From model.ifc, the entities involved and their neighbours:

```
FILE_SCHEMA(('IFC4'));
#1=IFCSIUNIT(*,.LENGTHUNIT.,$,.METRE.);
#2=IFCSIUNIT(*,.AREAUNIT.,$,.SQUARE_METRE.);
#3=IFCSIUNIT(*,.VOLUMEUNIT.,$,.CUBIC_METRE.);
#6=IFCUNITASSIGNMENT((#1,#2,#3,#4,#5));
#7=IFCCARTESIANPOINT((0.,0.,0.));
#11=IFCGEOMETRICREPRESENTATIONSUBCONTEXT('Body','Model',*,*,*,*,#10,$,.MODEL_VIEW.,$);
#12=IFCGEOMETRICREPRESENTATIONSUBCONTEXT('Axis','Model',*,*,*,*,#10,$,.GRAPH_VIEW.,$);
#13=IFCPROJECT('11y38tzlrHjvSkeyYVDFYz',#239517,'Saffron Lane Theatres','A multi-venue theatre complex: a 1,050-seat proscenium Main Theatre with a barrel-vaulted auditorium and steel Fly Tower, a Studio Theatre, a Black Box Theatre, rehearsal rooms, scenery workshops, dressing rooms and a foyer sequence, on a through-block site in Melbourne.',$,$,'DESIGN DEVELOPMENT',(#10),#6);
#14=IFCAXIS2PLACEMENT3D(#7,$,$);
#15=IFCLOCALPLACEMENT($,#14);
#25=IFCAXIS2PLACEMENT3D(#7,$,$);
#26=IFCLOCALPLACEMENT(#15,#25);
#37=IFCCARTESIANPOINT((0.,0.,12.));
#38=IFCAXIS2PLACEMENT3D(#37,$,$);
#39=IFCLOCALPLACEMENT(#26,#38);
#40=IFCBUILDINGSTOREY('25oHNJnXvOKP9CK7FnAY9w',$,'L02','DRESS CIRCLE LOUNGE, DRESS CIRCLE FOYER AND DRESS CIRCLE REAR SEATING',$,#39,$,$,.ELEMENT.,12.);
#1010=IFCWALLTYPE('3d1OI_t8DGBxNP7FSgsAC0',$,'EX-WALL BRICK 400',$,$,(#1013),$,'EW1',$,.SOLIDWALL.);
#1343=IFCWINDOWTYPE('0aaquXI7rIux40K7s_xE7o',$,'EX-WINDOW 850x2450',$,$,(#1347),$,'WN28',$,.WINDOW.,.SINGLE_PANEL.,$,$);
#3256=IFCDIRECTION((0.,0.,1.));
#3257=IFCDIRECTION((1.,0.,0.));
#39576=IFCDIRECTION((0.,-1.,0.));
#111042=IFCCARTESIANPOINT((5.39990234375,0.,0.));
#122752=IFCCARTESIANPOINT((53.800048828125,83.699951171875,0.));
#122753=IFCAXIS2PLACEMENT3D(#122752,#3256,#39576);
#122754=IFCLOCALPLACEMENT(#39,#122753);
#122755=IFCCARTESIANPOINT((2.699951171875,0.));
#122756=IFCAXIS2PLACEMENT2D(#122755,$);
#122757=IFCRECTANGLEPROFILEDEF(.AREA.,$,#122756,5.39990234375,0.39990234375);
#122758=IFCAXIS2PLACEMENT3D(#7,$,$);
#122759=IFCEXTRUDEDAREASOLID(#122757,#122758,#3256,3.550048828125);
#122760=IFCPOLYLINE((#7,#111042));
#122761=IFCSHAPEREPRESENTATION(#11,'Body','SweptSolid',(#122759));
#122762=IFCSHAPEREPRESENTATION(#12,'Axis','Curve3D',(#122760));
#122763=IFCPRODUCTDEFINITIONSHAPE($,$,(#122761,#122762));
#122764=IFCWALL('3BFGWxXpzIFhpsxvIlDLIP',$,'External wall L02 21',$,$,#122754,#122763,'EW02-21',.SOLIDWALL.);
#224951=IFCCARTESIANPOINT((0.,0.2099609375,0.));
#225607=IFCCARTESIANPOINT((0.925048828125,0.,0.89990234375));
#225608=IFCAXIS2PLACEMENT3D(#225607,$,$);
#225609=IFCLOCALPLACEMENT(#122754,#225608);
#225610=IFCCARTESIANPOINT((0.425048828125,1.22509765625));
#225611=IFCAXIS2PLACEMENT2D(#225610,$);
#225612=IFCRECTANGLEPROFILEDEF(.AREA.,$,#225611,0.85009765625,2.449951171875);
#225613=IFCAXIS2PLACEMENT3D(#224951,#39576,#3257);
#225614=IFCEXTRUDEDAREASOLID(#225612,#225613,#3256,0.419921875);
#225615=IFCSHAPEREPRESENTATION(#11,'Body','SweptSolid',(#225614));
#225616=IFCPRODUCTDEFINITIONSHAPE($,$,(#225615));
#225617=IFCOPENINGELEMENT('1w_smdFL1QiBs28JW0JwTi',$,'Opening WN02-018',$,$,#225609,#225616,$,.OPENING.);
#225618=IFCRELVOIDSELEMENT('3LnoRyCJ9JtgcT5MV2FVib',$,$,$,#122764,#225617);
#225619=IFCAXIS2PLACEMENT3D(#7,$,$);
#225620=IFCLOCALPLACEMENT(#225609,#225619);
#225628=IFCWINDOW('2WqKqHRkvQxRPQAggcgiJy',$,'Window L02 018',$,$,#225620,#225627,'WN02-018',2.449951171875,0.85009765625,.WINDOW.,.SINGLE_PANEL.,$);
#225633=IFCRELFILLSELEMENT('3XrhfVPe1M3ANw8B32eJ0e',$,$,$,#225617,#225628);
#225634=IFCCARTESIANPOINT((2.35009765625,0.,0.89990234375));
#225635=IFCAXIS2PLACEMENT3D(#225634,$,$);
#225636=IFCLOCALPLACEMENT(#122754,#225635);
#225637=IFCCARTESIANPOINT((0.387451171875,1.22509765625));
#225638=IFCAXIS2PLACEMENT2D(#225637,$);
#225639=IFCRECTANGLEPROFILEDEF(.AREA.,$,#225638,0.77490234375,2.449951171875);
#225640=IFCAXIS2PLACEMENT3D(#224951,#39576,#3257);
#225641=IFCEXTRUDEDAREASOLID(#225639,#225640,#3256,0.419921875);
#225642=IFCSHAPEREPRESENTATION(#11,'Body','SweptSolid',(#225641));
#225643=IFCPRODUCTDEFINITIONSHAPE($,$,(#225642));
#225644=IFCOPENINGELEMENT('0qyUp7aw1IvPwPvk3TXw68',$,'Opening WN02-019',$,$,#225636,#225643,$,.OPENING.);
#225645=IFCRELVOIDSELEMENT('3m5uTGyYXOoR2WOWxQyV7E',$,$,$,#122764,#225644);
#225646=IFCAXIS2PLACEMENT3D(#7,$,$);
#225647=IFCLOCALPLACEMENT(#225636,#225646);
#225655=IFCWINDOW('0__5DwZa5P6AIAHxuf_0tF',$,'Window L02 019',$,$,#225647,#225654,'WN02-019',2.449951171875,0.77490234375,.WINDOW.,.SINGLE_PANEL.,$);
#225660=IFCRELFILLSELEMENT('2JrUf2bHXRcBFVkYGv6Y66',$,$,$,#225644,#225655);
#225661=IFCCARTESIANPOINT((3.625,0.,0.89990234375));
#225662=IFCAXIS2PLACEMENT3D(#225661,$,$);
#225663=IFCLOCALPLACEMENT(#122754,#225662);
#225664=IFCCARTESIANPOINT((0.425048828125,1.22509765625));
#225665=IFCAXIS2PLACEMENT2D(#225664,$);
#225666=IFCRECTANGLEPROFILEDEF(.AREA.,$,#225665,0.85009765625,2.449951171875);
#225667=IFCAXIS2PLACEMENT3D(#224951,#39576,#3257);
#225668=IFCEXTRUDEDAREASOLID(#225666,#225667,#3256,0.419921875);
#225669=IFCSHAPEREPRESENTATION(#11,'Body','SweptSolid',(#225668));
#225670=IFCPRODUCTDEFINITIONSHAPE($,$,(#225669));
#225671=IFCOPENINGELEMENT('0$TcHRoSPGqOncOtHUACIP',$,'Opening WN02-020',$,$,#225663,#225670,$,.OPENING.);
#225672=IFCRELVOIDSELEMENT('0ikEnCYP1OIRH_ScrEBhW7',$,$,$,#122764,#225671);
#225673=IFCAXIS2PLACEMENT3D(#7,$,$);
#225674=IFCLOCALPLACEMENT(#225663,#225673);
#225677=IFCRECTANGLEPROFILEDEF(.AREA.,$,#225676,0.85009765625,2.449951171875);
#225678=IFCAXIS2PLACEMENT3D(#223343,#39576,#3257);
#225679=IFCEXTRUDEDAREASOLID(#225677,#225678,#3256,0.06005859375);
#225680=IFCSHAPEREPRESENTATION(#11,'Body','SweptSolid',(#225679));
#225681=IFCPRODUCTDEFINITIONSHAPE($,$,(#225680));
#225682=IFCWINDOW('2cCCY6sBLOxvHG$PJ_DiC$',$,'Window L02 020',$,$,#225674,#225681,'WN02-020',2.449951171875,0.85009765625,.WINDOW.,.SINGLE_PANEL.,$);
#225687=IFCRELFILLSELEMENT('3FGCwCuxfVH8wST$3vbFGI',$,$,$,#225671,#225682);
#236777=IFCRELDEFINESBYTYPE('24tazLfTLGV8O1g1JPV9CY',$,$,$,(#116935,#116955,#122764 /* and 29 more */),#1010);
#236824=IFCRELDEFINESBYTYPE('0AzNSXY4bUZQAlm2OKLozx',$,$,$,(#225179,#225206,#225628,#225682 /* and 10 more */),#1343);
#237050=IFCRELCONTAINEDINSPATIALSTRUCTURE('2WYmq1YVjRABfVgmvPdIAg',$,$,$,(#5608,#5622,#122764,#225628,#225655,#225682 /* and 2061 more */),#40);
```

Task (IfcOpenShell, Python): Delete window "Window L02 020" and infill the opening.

```python
import ifcopenshell
import ifcopenshell.api.feature
import ifcopenshell.api.root
import ifcopenshell.geom
import ifcopenshell.util.shape

model = ifcopenshell.open("model.ifc")
settings = ifcopenshell.geom.settings()


def volume(element):
    """Net volume in cubic metres, openings subtracted."""
    shape = ifcopenshell.geom.create_shape(settings, element)
    return ifcopenshell.util.shape.get_volume(shape.geometry)


window = model.by_guid("2cCCY6sBLOxvHG$PJ_DiC$")
opening = window.FillsVoids[0].RelatingOpeningElement
wall = opening.VoidsElements[0].RelatingBuildingElement
before = volume(wall)

ifcopenshell.api.root.remove_product(model, product=window)
ifcopenshell.api.feature.remove_feature(model, feature=opening)

after = volume(wall)

print(f"wall volume {before:.3f} -> {after:.3f} m3")

model.write("model_updated.ifc")
```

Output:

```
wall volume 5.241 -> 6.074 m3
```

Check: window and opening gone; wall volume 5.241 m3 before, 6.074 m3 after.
